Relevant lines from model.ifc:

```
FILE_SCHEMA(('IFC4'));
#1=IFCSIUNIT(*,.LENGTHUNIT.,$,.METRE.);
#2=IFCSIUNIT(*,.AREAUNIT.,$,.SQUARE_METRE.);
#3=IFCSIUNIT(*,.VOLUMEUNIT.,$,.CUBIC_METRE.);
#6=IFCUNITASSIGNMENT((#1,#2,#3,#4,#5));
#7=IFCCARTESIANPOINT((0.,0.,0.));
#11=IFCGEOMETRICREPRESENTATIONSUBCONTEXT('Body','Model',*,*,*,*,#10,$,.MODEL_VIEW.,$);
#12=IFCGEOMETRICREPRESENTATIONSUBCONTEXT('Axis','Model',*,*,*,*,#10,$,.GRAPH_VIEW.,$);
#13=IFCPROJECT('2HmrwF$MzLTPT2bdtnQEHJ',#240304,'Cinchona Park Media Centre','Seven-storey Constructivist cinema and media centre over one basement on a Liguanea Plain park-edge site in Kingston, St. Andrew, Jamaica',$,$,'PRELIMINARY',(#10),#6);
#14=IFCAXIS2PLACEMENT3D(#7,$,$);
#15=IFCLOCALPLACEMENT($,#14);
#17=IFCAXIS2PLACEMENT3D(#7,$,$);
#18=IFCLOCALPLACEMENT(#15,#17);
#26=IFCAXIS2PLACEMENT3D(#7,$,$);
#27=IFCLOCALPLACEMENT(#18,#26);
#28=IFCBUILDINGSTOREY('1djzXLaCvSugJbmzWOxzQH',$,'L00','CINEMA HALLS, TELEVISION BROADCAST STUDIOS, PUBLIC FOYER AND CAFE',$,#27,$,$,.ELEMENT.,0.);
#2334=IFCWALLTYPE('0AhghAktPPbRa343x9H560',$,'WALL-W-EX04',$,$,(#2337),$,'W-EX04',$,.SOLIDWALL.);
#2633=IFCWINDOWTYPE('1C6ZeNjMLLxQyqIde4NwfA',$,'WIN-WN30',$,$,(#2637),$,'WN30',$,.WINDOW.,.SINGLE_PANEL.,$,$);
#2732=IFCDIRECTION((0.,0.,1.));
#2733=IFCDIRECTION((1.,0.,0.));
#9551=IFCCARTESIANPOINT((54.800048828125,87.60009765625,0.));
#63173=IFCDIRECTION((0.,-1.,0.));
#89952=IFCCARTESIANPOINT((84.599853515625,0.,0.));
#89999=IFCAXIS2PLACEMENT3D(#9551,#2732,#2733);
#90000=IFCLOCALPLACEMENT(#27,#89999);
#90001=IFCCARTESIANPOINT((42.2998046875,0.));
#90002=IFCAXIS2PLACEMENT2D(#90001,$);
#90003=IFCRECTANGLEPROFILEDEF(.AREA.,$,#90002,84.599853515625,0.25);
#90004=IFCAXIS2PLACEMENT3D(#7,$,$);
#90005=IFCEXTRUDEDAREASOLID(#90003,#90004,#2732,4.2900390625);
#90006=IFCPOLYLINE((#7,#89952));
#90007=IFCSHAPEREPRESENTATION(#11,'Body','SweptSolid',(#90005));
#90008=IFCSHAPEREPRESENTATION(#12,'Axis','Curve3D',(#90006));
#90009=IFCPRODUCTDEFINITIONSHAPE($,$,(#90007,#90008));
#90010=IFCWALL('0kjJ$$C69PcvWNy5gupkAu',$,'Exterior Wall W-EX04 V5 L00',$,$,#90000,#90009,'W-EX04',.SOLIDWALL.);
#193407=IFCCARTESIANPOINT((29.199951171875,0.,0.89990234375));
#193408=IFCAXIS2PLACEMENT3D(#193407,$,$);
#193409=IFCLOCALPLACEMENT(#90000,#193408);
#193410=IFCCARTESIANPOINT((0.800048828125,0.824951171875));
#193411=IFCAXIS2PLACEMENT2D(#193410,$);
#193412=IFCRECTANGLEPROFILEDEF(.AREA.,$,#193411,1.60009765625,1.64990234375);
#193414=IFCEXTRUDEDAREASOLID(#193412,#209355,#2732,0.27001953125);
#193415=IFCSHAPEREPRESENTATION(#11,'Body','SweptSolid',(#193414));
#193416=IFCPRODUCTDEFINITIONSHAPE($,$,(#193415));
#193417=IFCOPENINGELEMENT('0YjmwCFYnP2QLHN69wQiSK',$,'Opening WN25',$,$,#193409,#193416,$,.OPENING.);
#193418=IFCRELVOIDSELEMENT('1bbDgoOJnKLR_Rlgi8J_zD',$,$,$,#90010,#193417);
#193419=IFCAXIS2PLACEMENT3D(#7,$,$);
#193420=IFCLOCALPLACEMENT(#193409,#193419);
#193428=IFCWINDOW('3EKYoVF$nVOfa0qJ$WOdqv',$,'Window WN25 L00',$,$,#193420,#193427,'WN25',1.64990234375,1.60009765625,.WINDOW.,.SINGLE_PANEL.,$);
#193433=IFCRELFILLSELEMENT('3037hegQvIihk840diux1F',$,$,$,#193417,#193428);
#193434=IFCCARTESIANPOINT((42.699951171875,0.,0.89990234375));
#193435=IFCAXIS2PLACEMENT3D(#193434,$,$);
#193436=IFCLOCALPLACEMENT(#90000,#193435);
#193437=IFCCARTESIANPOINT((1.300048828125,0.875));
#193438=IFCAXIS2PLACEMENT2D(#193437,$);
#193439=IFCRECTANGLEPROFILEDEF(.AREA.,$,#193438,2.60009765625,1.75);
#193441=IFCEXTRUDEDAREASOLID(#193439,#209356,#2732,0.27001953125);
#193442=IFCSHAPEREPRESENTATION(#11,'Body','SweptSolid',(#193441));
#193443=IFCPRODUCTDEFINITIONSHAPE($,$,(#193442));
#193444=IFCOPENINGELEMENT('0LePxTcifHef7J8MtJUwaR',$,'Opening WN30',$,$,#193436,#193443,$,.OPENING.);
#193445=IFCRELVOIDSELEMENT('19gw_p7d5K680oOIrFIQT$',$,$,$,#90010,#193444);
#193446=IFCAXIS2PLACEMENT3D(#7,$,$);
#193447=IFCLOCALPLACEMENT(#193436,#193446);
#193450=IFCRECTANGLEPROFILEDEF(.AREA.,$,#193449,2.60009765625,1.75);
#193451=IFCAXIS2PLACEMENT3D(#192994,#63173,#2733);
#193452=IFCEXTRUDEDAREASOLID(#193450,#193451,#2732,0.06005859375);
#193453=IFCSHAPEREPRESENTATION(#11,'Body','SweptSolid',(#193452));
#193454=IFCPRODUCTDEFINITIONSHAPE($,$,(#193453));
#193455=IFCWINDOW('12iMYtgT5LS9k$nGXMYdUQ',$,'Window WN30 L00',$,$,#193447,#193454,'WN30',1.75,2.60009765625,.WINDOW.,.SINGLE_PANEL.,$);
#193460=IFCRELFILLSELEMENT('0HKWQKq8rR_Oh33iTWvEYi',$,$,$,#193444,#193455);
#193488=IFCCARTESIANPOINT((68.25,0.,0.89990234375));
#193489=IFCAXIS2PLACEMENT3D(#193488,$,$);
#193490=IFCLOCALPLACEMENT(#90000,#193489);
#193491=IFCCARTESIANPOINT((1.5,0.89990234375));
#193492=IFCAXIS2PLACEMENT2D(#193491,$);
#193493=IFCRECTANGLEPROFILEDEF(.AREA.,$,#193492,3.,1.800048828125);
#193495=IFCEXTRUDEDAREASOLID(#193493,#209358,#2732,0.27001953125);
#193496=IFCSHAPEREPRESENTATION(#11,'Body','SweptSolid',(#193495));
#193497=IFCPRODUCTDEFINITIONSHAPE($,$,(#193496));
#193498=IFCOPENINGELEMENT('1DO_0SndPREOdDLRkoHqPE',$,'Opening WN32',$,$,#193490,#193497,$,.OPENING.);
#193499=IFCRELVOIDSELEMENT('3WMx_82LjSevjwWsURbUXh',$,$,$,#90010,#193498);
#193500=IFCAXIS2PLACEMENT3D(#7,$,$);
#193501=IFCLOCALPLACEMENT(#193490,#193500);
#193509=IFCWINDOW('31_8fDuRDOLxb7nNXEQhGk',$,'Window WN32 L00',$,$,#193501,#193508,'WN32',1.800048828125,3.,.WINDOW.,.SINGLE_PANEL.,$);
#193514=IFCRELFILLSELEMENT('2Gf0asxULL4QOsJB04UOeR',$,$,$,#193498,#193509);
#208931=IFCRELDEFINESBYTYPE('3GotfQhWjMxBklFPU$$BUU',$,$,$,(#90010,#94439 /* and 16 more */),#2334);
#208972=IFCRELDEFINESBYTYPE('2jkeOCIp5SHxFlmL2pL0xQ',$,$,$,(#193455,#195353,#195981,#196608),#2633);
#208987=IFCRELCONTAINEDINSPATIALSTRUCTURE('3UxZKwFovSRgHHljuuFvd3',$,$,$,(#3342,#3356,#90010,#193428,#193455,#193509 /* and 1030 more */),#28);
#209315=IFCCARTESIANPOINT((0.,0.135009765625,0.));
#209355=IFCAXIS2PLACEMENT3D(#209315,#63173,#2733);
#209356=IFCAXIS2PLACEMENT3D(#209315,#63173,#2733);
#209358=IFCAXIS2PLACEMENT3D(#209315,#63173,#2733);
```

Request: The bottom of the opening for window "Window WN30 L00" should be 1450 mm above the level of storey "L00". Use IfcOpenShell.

```python
import numpy as np
import ifcopenshell
import ifcopenshell.api.geometry
import ifcopenshell.geom
import ifcopenshell.util.element
import ifcopenshell.util.placement
import ifcopenshell.util.shape
import ifcopenshell.util.unit

model = ifcopenshell.open("model.ifc")
unit_scale = ifcopenshell.util.unit.calculate_unit_scale(model)

window = model.by_guid("12iMYtgT5LS9k$nGXMYdUQ")
opening = window.FillsVoids[0].RelatingOpeningElement
storey = ifcopenshell.util.element.get_container(window, ifc_class="IfcBuildingStorey")
level = ifcopenshell.util.placement.get_local_placement(storey.ObjectPlacement)[2, 3]

# The opening's origin need not be at the sill, so measure its lowest point.
shape = ifcopenshell.geom.create_shape(ifcopenshell.geom.settings(), opening)
bottom = ifcopenshell.util.shape.get_shape_bottom_elevation(shape, shape.geometry) / unit_scale
dz = level + 1.45 / unit_scale - bottom

shift = np.array([0.0, 0.0, dz])
# The window is placed relative to its opening, so it follows when the opening moves.
matrix = ifcopenshell.util.placement.get_local_placement(opening.ObjectPlacement)
matrix[:3, 3] += shift
ifcopenshell.api.geometry.edit_object_placement(
    model, product=opening, matrix=matrix, is_si=False, should_transform_children=True
)

print(f"moved by {dz * unit_scale:+.3f} m")

model.write("model_updated.ifc")
```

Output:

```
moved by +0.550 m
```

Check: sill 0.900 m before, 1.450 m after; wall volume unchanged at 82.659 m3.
